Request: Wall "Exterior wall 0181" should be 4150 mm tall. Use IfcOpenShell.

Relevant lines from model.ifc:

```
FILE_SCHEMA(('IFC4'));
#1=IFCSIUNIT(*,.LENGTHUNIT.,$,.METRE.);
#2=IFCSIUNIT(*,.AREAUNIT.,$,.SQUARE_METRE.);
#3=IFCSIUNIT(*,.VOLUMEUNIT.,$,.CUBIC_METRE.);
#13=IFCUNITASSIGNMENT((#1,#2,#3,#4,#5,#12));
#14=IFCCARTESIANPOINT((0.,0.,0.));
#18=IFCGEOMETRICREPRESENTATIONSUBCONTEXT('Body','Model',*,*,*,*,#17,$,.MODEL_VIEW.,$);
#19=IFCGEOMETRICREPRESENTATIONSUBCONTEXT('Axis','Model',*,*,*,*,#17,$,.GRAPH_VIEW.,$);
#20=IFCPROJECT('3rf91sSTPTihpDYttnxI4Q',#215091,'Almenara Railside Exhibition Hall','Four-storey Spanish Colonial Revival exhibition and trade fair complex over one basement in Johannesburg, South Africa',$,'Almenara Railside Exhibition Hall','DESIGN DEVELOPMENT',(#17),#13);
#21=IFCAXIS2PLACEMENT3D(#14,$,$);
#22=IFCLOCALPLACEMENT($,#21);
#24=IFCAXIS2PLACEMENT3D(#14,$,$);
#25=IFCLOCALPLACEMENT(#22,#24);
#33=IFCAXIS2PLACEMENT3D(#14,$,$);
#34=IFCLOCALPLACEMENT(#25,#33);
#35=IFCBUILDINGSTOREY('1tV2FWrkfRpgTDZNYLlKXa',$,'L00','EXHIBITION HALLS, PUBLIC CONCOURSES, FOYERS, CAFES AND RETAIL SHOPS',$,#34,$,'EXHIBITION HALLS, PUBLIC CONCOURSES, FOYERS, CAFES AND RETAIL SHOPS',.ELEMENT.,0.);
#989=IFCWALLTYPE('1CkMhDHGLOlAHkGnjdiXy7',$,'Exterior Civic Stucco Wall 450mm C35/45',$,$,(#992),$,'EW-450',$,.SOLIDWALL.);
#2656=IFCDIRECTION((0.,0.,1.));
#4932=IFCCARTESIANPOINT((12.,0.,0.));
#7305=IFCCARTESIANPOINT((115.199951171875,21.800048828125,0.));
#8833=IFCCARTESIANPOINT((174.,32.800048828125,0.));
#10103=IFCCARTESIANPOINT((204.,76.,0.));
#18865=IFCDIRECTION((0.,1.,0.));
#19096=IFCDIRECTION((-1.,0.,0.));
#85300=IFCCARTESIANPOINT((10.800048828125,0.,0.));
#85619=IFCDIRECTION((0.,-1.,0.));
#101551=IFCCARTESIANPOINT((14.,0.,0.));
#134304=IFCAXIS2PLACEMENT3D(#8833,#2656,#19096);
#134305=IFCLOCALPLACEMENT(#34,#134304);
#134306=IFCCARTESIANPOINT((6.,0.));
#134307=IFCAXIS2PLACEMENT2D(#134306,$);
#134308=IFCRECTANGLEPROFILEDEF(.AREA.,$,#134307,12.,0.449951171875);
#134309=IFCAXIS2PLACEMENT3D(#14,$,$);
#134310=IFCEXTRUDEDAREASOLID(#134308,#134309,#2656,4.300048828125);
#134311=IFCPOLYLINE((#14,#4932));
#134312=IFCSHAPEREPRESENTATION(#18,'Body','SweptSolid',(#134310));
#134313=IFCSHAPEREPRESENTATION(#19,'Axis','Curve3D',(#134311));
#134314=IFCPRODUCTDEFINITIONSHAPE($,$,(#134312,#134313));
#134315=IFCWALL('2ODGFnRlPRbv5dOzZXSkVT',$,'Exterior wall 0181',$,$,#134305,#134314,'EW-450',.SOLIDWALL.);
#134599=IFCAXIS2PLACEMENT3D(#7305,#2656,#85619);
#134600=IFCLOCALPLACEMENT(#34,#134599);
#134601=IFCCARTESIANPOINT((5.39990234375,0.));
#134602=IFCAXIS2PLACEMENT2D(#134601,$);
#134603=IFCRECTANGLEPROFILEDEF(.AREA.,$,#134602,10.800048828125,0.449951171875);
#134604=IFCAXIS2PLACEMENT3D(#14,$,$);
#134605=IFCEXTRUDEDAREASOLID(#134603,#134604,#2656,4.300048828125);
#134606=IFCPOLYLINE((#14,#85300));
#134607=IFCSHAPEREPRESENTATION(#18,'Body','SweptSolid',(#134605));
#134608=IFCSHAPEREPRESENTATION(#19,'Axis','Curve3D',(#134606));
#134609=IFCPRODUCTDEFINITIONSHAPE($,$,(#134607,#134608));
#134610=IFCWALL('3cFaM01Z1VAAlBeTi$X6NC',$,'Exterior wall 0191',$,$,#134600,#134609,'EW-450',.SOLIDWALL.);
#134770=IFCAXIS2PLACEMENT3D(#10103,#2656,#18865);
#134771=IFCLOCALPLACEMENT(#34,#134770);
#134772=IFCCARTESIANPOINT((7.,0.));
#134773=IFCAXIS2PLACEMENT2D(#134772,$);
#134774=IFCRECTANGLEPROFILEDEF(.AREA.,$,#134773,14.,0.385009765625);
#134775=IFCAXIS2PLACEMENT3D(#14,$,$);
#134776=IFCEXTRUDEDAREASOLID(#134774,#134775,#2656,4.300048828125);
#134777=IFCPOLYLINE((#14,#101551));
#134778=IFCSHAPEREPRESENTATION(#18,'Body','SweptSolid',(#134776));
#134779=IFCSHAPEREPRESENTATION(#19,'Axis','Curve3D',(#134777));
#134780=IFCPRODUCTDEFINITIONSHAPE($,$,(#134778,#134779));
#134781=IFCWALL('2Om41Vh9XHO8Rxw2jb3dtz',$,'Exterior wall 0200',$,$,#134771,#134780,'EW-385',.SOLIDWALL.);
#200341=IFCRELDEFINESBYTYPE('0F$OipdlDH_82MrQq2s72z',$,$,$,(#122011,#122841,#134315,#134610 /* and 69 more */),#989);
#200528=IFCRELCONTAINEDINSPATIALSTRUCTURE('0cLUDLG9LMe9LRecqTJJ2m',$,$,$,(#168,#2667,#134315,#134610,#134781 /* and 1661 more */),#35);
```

```python
import ifcopenshell
import ifcopenshell.geom
import ifcopenshell.util.representation
import ifcopenshell.util.shape

model = ifcopenshell.open("model.ifc")
settings = ifcopenshell.geom.settings()


def volume(element):
    """Net volume in cubic metres, openings subtracted."""
    shape = ifcopenshell.geom.create_shape(settings, element)
    return ifcopenshell.util.shape.get_volume(shape.geometry)


wall = model.by_guid("2ODGFnRlPRbv5dOzZXSkVT")
before = volume(wall)

body = ifcopenshell.util.representation.get_representation(wall, "Model", "Body")
solid = body.Items[0]
old_height = solid.Depth
solid.Depth = 4.15
after = volume(wall)

print(f"height {old_height:g} -> {solid.Depth:g}, volume {before:.3f} -> {after:.3f} m3")

model.write("model_updated.ifc")
```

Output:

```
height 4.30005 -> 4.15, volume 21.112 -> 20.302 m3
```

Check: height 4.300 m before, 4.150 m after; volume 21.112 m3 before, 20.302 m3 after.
